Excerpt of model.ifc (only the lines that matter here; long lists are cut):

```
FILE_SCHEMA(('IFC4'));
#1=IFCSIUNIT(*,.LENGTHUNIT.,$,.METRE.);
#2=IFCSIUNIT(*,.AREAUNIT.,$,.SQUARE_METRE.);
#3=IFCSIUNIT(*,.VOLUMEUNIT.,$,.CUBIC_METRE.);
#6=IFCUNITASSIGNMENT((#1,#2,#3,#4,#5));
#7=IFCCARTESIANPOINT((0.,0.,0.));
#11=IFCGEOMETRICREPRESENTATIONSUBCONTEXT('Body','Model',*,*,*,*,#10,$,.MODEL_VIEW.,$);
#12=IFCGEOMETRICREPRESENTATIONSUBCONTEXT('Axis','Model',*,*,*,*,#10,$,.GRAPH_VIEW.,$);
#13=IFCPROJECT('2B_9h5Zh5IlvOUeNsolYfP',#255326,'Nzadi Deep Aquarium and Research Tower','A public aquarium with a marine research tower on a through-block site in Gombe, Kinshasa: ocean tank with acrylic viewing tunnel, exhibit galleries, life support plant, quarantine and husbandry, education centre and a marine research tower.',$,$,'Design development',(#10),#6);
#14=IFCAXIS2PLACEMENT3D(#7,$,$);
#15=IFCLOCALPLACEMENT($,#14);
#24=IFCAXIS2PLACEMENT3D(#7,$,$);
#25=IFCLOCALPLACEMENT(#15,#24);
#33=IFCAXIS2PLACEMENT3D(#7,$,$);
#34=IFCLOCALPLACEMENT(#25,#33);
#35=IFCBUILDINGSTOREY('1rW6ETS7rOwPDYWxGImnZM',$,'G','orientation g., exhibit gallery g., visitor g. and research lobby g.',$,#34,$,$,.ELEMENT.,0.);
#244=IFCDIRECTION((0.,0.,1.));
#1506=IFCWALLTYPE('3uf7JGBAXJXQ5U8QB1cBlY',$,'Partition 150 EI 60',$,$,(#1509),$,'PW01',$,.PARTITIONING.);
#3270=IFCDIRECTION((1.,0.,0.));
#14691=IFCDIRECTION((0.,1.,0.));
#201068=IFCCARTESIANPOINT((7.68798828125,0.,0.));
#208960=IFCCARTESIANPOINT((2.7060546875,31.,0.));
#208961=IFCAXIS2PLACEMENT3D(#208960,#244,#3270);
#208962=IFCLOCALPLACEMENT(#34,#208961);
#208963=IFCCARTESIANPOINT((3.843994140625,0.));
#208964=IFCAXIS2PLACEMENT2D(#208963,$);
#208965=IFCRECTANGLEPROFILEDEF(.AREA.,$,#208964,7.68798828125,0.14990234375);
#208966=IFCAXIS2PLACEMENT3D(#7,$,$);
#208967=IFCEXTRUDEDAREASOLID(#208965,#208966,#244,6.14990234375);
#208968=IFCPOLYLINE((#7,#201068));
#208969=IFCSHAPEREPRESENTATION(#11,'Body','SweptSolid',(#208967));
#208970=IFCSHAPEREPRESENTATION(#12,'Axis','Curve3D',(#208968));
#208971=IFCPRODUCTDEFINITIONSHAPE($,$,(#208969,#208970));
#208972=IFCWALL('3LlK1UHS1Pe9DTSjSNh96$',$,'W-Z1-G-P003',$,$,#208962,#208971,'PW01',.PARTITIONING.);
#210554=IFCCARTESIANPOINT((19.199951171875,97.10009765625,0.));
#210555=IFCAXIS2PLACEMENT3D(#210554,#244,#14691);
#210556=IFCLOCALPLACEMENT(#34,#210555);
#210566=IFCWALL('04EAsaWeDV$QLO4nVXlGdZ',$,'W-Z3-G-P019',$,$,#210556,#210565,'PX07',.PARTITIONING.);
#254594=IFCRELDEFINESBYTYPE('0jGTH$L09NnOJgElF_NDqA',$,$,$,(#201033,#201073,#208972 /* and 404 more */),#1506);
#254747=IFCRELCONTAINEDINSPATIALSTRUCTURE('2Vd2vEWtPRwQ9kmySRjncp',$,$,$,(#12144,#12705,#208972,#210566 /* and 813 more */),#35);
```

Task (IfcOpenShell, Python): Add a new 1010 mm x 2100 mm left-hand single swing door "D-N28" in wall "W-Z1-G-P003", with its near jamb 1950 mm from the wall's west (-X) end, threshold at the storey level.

```python
import numpy as np
import ifcopenshell
import ifcopenshell.api.feature
import ifcopenshell.api.geometry
import ifcopenshell.api.root
import ifcopenshell.api.spatial
import ifcopenshell.geom
import ifcopenshell.util.element
import ifcopenshell.util.placement
import ifcopenshell.util.representation
import ifcopenshell.util.shape
import ifcopenshell.util.unit

model = ifcopenshell.open("model.ifc")
unit_scale = ifcopenshell.util.unit.calculate_unit_scale(model)
settings = ifcopenshell.geom.settings()


def volume(element):
    """Net volume in cubic metres, openings subtracted."""
    shape = ifcopenshell.geom.create_shape(settings, element)
    return ifcopenshell.util.shape.get_volume(shape.geometry)


wall = model.by_guid("3LlK1UHS1Pe9DTSjSNh96$")
storey = ifcopenshell.util.element.get_container(wall, ifc_class="IfcBuildingStorey")
context = ifcopenshell.util.representation.get_context(model, "Model", "Body", "MODEL_VIEW")
before = volume(wall)

width, height, from_end, sill = 1.01, 2.1, 1.95, 0.0  # metres

# The wall runs along its own X axis, and the end named is its -X end.
wall_shape = ifcopenshell.geom.create_shape(settings, wall)
x, y, z = ifcopenshell.util.shape.get_vertices(wall_shape.geometry).T
start = x.min() + from_end
face, thickness = float(y.min()), float(y.max() - y.min())
wall_matrix = ifcopenshell.util.placement.get_local_placement(wall.ObjectPlacement)
level = ifcopenshell.util.placement.get_local_placement(storey.ObjectPlacement)[2, 3]


def in_wall(x, y):
    """Placement at x, y metres in the wall's axes, at sill height."""
    matrix = wall_matrix.copy()
    matrix[:, 3] = wall_matrix @ np.array([x / unit_scale, y / unit_scale, 0.0, 1.0])
    matrix[2, 3] = level + sill / unit_scale
    return matrix


# Opening: a box that overshoots both wall faces by 50 mm.
opening = ifcopenshell.api.root.create_entity(model, ifc_class="IfcOpeningElement", predefined_type="OPENING")
box = ifcopenshell.api.geometry.add_wall_representation(
    model, context=context, length=width, height=height, thickness=thickness + 0.1
)
ifcopenshell.api.geometry.assign_representation(model, product=opening, representation=box)
ifcopenshell.api.geometry.edit_object_placement(model, product=opening, matrix=in_wall(start, face - 0.05), is_si=False)
ifcopenshell.api.feature.add_feature(model, feature=opening, element=wall)

door = ifcopenshell.api.root.create_entity(model, ifc_class="IfcDoor", name="D-N28", predefined_type="DOOR")
door.OverallWidth, door.OverallHeight = width / unit_scale, height / unit_scale
door.OperationType = "SINGLE_SWING_LEFT"
body = ifcopenshell.api.geometry.add_door_representation(
    model,
    context=context,
    overall_width=door.OverallWidth,
    overall_height=door.OverallHeight,
    operation_type="SINGLE_SWING_LEFT",
    lining_properties={"LiningDepth": thickness / unit_scale, "ThresholdDepth": thickness / unit_scale},
)
ifcopenshell.api.geometry.assign_representation(model, product=door, representation=body)
ifcopenshell.api.spatial.assign_container(model, products=[door], relating_structure=storey)
ifcopenshell.api.feature.add_filling(model, opening=opening, element=door)

# The lining spans the wall, so the door starts at the wall face.
ifcopenshell.api.geometry.edit_object_placement(model, product=door, matrix=in_wall(start, face), is_si=False)

after = volume(wall)

print(f"wall volume {before:.3f} -> {after:.3f} m3")

model.write("model_v2.ifc")
```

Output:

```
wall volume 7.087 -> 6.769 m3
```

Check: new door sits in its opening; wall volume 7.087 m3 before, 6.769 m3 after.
